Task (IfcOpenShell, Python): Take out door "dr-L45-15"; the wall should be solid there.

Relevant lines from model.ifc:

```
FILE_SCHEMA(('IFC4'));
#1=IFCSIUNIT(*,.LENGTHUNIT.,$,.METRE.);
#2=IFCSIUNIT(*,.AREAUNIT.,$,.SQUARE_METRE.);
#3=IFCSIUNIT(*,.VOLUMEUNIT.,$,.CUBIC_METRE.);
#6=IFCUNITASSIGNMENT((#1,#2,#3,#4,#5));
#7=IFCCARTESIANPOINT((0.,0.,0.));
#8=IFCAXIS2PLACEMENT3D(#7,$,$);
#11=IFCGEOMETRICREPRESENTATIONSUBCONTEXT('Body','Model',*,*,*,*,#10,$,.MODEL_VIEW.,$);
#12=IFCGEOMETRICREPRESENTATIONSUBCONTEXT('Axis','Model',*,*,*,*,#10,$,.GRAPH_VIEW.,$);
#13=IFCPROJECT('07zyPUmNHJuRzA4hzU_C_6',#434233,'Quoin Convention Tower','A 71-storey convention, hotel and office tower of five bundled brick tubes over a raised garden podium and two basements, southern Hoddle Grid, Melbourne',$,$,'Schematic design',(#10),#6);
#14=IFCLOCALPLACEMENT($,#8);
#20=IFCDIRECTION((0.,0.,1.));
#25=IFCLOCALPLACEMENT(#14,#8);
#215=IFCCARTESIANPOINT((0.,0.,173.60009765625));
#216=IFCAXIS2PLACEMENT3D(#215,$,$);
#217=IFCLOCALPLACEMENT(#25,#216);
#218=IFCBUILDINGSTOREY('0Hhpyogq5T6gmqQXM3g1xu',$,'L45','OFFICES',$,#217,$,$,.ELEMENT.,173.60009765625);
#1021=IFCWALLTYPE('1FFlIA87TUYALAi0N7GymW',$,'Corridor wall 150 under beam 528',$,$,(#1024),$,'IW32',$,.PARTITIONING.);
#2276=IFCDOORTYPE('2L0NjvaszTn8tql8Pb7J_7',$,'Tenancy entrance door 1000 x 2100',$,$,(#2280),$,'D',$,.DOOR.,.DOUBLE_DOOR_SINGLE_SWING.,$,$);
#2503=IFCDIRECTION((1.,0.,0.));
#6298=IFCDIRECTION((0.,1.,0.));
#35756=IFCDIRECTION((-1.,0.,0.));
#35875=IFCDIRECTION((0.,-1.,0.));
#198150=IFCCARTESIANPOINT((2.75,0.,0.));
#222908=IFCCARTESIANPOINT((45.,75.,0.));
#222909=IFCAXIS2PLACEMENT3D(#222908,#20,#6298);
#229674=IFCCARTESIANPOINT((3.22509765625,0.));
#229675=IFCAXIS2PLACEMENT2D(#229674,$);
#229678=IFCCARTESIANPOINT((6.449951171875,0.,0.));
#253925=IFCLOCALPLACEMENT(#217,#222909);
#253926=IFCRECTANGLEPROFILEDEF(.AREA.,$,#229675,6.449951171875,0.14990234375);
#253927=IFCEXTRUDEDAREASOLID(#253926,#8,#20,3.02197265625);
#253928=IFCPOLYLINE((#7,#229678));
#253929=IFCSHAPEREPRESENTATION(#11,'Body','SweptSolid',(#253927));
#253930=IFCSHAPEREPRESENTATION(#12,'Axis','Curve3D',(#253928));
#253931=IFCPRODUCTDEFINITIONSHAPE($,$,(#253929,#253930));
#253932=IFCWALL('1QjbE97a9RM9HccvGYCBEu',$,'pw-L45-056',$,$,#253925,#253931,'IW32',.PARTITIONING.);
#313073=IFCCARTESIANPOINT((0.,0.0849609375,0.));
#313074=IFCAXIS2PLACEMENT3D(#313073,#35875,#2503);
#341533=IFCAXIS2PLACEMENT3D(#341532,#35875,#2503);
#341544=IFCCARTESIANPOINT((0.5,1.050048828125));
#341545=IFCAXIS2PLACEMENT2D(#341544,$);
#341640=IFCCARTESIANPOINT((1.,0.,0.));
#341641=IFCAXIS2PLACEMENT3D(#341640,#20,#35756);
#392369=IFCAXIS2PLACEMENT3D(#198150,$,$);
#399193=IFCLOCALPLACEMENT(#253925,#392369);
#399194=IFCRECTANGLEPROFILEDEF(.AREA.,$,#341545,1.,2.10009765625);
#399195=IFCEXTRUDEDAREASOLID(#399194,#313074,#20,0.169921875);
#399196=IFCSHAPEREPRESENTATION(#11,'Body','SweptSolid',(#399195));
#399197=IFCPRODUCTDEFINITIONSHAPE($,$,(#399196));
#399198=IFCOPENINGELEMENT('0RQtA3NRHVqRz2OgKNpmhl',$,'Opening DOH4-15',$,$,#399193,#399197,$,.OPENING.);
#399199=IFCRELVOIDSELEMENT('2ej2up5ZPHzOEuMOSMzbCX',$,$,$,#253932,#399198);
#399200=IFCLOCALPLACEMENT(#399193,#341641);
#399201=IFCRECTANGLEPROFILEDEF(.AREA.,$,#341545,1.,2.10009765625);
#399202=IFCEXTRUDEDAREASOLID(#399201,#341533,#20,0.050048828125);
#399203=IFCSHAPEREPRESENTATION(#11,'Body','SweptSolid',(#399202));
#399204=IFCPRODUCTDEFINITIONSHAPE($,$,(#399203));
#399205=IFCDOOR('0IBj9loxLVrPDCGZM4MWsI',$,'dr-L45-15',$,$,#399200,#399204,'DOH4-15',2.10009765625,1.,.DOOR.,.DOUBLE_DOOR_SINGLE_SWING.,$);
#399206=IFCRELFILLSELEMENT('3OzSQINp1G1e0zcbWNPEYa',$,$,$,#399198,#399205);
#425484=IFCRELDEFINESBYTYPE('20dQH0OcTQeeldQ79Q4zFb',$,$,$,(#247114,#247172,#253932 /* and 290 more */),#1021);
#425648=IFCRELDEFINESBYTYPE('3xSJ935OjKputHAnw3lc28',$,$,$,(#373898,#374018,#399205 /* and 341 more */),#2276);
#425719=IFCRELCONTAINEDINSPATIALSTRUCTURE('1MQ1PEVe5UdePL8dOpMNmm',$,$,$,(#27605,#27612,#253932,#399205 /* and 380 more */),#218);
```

```python
import ifcopenshell
import ifcopenshell.api.feature
import ifcopenshell.api.root
import ifcopenshell.geom
import ifcopenshell.util.shape

model = ifcopenshell.open("model.ifc")
settings = ifcopenshell.geom.settings()


def volume(element):
    """Net volume in cubic metres, openings subtracted."""
    shape = ifcopenshell.geom.create_shape(settings, element)
    return ifcopenshell.util.shape.get_volume(shape.geometry)


door = model.by_guid("0IBj9loxLVrPDCGZM4MWsI")
opening = door.FillsVoids[0].RelatingOpeningElement
wall = opening.VoidsElements[0].RelatingBuildingElement
before = volume(wall)

ifcopenshell.api.root.remove_product(model, product=door)
ifcopenshell.api.feature.remove_feature(model, feature=opening)

after = volume(wall)

print(f"wall volume {before:.3f} -> {after:.3f} m3")

model.write("model-out.ifc")
```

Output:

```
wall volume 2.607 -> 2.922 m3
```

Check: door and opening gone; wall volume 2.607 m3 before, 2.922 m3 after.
